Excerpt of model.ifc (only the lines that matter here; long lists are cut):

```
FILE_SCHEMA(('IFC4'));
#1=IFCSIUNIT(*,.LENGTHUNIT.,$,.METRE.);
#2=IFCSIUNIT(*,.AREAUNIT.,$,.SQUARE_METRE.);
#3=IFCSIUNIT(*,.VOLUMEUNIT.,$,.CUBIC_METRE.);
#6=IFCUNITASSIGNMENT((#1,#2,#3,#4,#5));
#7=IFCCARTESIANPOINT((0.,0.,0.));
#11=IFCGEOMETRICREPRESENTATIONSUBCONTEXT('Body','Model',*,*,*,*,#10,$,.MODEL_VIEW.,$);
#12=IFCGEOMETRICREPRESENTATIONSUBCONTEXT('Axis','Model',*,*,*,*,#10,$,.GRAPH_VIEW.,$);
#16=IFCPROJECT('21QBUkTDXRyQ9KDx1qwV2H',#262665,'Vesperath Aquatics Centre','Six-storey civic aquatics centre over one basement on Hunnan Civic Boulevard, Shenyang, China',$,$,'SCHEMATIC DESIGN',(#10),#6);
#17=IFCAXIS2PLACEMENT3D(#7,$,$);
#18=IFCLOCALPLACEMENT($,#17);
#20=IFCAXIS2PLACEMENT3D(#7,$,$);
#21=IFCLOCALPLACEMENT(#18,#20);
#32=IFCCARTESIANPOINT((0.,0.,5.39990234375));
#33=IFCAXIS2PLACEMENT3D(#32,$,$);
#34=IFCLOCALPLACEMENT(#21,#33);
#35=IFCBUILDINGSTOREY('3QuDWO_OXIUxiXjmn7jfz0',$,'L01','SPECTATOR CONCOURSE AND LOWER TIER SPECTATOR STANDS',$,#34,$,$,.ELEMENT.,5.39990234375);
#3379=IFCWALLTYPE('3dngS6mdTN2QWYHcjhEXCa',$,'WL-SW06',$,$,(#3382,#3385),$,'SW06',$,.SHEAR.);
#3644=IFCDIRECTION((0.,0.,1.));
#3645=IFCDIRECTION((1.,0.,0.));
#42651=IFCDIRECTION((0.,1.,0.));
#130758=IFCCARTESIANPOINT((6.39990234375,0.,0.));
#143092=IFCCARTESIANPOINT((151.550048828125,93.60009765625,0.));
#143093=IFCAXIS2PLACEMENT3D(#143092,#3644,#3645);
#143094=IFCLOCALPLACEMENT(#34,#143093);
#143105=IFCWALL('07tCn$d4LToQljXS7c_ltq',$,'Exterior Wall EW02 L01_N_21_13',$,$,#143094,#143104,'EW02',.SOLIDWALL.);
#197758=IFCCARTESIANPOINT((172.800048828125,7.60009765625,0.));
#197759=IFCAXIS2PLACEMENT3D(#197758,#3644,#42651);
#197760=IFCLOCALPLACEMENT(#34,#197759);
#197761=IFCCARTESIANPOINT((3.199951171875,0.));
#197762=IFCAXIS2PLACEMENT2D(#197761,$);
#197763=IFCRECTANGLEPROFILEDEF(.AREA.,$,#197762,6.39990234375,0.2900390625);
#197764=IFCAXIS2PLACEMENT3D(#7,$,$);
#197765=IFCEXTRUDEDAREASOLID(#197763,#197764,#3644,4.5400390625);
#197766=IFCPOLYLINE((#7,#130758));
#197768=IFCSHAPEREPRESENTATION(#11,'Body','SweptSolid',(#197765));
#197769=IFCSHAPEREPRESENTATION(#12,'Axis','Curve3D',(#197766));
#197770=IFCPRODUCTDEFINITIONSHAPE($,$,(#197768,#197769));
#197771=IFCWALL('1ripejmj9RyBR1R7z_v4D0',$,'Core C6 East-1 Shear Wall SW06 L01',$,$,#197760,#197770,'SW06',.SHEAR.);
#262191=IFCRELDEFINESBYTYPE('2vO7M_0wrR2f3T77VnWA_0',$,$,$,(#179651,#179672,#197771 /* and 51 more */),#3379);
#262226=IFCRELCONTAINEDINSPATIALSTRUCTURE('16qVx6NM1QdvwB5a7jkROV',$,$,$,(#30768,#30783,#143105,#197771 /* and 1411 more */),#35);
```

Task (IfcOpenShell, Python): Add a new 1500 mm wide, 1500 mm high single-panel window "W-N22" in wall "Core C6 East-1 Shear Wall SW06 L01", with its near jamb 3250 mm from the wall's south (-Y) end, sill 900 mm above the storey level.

```python
import numpy as np
import ifcopenshell
import ifcopenshell.api.feature
import ifcopenshell.api.geometry
import ifcopenshell.api.root
import ifcopenshell.api.spatial
import ifcopenshell.geom
import ifcopenshell.util.element
import ifcopenshell.util.placement
import ifcopenshell.util.representation
import ifcopenshell.util.shape
import ifcopenshell.util.unit

model = ifcopenshell.open("model.ifc")
unit_scale = ifcopenshell.util.unit.calculate_unit_scale(model)
settings = ifcopenshell.geom.settings()


def volume(element):
    """Net volume in cubic metres, openings subtracted."""
    shape = ifcopenshell.geom.create_shape(settings, element)
    return ifcopenshell.util.shape.get_volume(shape.geometry)


wall = model.by_id(197771)
storey = ifcopenshell.util.element.get_container(wall, ifc_class="IfcBuildingStorey")
context = ifcopenshell.util.representation.get_context(model, "Model", "Body", "MODEL_VIEW")
before = volume(wall)

width, height, from_end, sill = 1.5, 1.5, 3.25, 0.9  # metres

# The wall runs along its own X axis, and the end named is its -X end.
wall_shape = ifcopenshell.geom.create_shape(settings, wall)
x, y, z = ifcopenshell.util.shape.get_vertices(wall_shape.geometry).T
start = x.min() + from_end
face, thickness = float(y.min()), float(y.max() - y.min())
wall_matrix = ifcopenshell.util.placement.get_local_placement(wall.ObjectPlacement)
level = ifcopenshell.util.placement.get_local_placement(storey.ObjectPlacement)[2, 3]


def in_wall(x, y):
    """Placement at x, y metres in the wall's axes, at sill height."""
    matrix = wall_matrix.copy()
    matrix[:, 3] = wall_matrix @ np.array([x / unit_scale, y / unit_scale, 0.0, 1.0])
    matrix[2, 3] = level + sill / unit_scale
    return matrix


# Opening: a box that overshoots both wall faces by 50 mm.
opening = ifcopenshell.api.root.create_entity(model, ifc_class="IfcOpeningElement", predefined_type="OPENING")
box = ifcopenshell.api.geometry.add_wall_representation(
    model, context=context, length=width, height=height, thickness=thickness + 0.1
)
ifcopenshell.api.geometry.assign_representation(model, product=opening, representation=box)
ifcopenshell.api.geometry.edit_object_placement(model, product=opening, matrix=in_wall(start, face - 0.05), is_si=False)
ifcopenshell.api.feature.add_feature(model, feature=opening, element=wall)

window = ifcopenshell.api.root.create_entity(model, ifc_class="IfcWindow", name="W-N22", predefined_type="WINDOW")
window.OverallWidth, window.OverallHeight = width / unit_scale, height / unit_scale
window.PartitioningType = "SINGLE_PANEL"
body = ifcopenshell.api.geometry.add_window_representation(
    model,
    context=context,
    overall_width=window.OverallWidth,
    overall_height=window.OverallHeight,
    partition_type="SINGLE_PANEL",
)
ifcopenshell.api.geometry.assign_representation(model, product=window, representation=body)
ifcopenshell.api.spatial.assign_container(model, products=[window], relating_structure=storey)
ifcopenshell.api.feature.add_filling(model, opening=opening, element=window)

# Centre the window in the wall's thickness.
ifcopenshell.api.geometry.edit_object_placement(model, product=window, matrix=in_wall(start, face), is_si=False)
window_shape = ifcopenshell.geom.create_shape(settings, window)
depth = ifcopenshell.util.shape.get_vertices(window_shape.geometry)[:, 1]
offset = face + thickness / 2 - (depth.min() + depth.max()) / 2
ifcopenshell.api.geometry.edit_object_placement(model, product=window, matrix=in_wall(start, offset), is_si=False)

after = volume(wall)

print(f"wall volume {before:.3f} -> {after:.3f} m3")

model.write("model_edited.ifc")
```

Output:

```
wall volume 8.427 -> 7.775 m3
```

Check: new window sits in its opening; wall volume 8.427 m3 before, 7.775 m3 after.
